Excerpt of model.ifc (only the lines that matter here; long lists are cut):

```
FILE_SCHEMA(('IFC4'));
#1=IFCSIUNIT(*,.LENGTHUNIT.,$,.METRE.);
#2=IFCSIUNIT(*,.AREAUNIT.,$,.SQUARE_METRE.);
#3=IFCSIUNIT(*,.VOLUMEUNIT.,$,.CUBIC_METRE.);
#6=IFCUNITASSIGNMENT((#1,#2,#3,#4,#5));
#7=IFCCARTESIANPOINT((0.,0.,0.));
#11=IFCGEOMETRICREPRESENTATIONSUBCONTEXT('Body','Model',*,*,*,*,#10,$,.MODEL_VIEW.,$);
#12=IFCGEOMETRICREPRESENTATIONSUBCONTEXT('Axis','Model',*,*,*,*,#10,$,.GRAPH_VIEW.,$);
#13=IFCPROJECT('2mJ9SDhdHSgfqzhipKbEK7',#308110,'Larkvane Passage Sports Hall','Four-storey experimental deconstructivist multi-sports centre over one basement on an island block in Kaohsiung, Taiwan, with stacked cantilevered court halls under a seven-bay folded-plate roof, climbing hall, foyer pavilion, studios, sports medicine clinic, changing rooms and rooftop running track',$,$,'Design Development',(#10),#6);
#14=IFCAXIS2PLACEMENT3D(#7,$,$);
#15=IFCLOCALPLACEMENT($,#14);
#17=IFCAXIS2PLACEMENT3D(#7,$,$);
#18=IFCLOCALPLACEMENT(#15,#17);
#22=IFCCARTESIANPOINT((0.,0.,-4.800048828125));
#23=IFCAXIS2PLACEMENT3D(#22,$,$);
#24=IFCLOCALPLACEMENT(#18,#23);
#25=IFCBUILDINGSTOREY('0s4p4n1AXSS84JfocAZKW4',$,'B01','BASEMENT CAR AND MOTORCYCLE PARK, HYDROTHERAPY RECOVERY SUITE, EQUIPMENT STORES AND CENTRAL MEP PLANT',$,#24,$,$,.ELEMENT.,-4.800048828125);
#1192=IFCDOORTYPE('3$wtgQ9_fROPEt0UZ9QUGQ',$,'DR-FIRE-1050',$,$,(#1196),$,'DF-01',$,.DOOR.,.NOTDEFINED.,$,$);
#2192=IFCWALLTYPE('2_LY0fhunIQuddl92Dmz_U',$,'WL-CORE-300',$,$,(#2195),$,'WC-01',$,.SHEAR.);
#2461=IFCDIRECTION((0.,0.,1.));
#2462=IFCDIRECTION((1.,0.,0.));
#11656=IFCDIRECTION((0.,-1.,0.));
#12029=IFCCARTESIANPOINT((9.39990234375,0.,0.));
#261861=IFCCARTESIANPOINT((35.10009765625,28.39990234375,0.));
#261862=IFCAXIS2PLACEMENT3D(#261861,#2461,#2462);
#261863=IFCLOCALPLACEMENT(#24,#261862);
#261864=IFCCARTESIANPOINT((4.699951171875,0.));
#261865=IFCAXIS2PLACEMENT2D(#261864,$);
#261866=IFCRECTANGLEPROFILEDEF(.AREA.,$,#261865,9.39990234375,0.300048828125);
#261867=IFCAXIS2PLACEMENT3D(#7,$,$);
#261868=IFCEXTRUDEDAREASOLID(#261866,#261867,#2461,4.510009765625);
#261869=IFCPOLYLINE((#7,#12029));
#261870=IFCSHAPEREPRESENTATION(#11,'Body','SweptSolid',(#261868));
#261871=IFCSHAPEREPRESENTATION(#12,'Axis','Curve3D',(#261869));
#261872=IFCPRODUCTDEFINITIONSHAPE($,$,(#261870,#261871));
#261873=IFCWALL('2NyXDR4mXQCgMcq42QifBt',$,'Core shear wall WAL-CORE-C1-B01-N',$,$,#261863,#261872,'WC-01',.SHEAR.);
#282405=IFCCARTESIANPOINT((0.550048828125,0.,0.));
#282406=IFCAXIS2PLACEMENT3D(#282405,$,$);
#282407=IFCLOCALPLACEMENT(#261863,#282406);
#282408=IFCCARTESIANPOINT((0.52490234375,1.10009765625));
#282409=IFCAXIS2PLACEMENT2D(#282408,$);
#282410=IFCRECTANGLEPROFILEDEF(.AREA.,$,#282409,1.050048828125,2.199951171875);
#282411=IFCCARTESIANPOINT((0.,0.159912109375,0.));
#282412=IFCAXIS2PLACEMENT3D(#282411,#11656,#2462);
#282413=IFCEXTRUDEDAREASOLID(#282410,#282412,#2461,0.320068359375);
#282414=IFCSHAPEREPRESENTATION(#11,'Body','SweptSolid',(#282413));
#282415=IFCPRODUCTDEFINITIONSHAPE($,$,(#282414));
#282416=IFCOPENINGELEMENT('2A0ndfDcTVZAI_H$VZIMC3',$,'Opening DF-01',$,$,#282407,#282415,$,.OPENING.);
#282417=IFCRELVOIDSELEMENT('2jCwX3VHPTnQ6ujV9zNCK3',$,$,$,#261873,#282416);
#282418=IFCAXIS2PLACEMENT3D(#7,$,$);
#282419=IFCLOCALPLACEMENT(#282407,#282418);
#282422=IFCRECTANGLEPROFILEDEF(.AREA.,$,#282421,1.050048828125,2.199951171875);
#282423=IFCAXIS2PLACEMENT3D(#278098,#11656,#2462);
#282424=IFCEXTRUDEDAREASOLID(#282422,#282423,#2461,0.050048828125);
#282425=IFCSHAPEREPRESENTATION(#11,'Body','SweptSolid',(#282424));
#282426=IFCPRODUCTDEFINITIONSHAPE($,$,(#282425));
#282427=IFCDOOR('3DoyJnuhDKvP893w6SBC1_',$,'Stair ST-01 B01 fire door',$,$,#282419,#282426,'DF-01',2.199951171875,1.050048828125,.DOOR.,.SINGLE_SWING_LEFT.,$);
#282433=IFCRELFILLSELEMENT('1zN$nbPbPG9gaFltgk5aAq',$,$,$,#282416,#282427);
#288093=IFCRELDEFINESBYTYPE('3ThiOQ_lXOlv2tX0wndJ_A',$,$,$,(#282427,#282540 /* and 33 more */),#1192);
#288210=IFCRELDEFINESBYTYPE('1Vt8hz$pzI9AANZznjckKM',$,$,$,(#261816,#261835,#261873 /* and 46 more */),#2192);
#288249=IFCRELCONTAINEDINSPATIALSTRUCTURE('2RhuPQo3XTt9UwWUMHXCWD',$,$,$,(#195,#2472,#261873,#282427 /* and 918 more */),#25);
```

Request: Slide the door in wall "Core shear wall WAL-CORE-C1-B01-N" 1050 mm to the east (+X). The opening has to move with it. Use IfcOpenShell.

```python
import ifcopenshell
import ifcopenshell.api.geometry
import ifcopenshell.util.placement

model = ifcopenshell.open("model.ifc")

door = model.by_guid("3DoyJnuhDKvP893w6SBC1_")
opening = door.FillsVoids[0].RelatingOpeningElement
wall = opening.VoidsElements[0].RelatingBuildingElement

wall_matrix = ifcopenshell.util.placement.get_local_placement(wall.ObjectPlacement)
shift = wall_matrix[:3, 0] * 1.05
before = ifcopenshell.util.placement.get_local_placement(door.ObjectPlacement)[:3, 3].copy()

# The door is placed relative to its opening, so it follows when the opening moves.
matrix = ifcopenshell.util.placement.get_local_placement(opening.ObjectPlacement)
matrix[:3, 3] += shift
ifcopenshell.api.geometry.edit_object_placement(
    model, product=opening, matrix=matrix, is_si=False, should_transform_children=True
)

after = ifcopenshell.util.placement.get_local_placement(door.ObjectPlacement)[:3, 3]
print("door moved by", (after - before).round(3) + 0.0)

model.write("model_edited.ifc")
```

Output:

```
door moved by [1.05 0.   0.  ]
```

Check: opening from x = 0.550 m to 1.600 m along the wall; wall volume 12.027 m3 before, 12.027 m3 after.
